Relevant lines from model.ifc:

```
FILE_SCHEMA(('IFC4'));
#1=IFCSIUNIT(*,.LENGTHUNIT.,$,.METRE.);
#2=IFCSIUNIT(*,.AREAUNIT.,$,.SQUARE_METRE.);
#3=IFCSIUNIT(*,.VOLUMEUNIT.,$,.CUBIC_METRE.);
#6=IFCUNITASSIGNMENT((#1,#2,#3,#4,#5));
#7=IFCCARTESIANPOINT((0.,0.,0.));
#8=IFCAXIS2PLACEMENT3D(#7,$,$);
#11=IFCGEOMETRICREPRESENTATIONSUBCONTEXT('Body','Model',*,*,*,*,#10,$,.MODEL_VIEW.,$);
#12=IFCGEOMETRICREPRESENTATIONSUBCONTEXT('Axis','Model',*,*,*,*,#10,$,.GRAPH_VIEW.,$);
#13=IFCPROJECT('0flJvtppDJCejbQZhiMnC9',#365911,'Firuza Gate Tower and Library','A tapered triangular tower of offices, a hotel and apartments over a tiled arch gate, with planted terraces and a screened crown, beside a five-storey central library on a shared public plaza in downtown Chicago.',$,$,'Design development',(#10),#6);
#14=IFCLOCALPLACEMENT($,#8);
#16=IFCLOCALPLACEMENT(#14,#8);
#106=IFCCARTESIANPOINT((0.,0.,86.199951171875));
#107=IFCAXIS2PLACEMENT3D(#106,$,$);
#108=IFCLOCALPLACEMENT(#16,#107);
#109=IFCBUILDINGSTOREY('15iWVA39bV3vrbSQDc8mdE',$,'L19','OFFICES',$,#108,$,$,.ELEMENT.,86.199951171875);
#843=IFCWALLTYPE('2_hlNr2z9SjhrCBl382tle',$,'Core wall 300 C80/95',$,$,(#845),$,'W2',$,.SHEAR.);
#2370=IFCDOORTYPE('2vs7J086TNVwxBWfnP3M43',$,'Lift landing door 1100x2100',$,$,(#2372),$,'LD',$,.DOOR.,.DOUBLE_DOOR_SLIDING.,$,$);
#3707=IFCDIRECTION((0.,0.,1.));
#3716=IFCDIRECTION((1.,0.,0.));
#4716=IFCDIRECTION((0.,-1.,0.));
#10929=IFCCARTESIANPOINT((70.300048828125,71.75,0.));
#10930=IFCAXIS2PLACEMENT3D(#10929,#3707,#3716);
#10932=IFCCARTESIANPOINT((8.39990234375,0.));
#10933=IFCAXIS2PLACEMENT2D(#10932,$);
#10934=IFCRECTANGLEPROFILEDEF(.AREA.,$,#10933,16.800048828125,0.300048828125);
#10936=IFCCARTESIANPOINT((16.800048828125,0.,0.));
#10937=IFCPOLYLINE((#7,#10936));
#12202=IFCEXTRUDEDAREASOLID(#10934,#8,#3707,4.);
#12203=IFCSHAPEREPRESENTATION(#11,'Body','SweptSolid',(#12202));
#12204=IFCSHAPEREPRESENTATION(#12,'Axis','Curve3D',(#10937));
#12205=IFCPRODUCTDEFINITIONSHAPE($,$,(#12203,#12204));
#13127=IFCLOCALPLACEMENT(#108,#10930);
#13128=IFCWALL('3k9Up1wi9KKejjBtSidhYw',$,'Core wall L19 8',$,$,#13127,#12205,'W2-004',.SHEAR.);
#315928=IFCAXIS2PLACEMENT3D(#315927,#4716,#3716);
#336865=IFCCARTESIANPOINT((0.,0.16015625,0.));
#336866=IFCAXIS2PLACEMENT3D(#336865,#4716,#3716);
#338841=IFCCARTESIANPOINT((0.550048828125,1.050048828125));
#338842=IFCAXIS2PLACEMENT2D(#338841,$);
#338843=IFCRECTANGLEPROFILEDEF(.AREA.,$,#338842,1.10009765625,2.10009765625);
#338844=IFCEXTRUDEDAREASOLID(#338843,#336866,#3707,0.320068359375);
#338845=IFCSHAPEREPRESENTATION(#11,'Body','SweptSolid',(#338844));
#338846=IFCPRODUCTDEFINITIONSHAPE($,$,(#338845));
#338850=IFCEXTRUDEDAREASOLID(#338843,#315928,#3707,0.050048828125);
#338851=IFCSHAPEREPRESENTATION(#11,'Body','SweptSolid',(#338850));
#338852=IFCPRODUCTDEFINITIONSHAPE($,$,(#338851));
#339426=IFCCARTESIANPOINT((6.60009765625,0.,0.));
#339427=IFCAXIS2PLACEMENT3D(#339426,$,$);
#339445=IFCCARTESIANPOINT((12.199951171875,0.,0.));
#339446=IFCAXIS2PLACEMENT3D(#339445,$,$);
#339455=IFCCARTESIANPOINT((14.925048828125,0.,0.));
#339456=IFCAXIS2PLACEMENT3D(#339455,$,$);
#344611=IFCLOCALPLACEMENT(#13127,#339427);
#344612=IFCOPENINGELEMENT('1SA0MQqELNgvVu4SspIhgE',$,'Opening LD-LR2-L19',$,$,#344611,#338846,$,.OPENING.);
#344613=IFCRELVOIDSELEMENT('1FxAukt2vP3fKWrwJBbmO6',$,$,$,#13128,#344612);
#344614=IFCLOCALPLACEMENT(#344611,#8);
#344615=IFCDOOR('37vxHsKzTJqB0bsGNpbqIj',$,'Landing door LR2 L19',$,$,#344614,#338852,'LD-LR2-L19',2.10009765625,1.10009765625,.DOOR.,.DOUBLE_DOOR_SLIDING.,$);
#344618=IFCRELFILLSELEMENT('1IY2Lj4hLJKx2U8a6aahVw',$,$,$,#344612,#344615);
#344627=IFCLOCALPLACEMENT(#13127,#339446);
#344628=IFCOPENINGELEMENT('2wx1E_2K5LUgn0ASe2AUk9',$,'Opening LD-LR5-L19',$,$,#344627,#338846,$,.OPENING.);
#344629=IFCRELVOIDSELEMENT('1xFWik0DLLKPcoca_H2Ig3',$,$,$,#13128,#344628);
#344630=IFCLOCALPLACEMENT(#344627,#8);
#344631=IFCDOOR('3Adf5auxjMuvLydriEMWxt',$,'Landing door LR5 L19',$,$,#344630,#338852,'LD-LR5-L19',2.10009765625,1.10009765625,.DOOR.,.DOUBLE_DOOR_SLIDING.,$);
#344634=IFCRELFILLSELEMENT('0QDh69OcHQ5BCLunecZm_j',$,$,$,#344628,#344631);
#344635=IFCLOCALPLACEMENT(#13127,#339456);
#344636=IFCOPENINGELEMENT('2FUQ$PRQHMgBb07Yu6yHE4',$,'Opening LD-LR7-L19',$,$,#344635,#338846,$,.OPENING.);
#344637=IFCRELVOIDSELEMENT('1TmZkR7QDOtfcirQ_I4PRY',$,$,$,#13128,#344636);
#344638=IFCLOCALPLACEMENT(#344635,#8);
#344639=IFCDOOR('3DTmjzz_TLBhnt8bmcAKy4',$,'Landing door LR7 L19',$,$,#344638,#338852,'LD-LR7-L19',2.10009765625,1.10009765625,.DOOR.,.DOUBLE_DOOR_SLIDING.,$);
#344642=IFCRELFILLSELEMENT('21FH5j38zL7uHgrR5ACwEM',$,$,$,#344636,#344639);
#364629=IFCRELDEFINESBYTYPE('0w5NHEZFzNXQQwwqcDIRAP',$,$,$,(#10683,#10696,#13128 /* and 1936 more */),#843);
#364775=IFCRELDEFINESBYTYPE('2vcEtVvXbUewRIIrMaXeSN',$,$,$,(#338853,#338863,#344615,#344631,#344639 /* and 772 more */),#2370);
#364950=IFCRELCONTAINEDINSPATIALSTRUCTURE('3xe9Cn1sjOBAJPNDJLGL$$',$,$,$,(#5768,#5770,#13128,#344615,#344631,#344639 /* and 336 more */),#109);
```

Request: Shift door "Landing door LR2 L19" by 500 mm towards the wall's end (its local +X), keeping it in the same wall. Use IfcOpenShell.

```python
import ifcopenshell
import ifcopenshell.api.geometry
import ifcopenshell.util.placement

model = ifcopenshell.open("model.ifc")

door = model.by_guid("37vxHsKzTJqB0bsGNpbqIj")
opening = door.FillsVoids[0].RelatingOpeningElement
wall = opening.VoidsElements[0].RelatingBuildingElement

wall_matrix = ifcopenshell.util.placement.get_local_placement(wall.ObjectPlacement)
shift = wall_matrix[:3, 0] * 0.5
before = ifcopenshell.util.placement.get_local_placement(door.ObjectPlacement)[:3, 3].copy()

# The door is placed relative to its opening, so it follows when the opening moves.
matrix = ifcopenshell.util.placement.get_local_placement(opening.ObjectPlacement)
matrix[:3, 3] += shift
ifcopenshell.api.geometry.edit_object_placement(
    model, product=opening, matrix=matrix, is_si=False, should_transform_children=True
)

after = ifcopenshell.util.placement.get_local_placement(door.ObjectPlacement)[:3, 3]
print("door moved by", (after - before).round(3) + 0.0)

model.write("model_v2.ifc")
```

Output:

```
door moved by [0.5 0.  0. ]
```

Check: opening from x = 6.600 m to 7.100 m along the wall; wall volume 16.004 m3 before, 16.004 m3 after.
